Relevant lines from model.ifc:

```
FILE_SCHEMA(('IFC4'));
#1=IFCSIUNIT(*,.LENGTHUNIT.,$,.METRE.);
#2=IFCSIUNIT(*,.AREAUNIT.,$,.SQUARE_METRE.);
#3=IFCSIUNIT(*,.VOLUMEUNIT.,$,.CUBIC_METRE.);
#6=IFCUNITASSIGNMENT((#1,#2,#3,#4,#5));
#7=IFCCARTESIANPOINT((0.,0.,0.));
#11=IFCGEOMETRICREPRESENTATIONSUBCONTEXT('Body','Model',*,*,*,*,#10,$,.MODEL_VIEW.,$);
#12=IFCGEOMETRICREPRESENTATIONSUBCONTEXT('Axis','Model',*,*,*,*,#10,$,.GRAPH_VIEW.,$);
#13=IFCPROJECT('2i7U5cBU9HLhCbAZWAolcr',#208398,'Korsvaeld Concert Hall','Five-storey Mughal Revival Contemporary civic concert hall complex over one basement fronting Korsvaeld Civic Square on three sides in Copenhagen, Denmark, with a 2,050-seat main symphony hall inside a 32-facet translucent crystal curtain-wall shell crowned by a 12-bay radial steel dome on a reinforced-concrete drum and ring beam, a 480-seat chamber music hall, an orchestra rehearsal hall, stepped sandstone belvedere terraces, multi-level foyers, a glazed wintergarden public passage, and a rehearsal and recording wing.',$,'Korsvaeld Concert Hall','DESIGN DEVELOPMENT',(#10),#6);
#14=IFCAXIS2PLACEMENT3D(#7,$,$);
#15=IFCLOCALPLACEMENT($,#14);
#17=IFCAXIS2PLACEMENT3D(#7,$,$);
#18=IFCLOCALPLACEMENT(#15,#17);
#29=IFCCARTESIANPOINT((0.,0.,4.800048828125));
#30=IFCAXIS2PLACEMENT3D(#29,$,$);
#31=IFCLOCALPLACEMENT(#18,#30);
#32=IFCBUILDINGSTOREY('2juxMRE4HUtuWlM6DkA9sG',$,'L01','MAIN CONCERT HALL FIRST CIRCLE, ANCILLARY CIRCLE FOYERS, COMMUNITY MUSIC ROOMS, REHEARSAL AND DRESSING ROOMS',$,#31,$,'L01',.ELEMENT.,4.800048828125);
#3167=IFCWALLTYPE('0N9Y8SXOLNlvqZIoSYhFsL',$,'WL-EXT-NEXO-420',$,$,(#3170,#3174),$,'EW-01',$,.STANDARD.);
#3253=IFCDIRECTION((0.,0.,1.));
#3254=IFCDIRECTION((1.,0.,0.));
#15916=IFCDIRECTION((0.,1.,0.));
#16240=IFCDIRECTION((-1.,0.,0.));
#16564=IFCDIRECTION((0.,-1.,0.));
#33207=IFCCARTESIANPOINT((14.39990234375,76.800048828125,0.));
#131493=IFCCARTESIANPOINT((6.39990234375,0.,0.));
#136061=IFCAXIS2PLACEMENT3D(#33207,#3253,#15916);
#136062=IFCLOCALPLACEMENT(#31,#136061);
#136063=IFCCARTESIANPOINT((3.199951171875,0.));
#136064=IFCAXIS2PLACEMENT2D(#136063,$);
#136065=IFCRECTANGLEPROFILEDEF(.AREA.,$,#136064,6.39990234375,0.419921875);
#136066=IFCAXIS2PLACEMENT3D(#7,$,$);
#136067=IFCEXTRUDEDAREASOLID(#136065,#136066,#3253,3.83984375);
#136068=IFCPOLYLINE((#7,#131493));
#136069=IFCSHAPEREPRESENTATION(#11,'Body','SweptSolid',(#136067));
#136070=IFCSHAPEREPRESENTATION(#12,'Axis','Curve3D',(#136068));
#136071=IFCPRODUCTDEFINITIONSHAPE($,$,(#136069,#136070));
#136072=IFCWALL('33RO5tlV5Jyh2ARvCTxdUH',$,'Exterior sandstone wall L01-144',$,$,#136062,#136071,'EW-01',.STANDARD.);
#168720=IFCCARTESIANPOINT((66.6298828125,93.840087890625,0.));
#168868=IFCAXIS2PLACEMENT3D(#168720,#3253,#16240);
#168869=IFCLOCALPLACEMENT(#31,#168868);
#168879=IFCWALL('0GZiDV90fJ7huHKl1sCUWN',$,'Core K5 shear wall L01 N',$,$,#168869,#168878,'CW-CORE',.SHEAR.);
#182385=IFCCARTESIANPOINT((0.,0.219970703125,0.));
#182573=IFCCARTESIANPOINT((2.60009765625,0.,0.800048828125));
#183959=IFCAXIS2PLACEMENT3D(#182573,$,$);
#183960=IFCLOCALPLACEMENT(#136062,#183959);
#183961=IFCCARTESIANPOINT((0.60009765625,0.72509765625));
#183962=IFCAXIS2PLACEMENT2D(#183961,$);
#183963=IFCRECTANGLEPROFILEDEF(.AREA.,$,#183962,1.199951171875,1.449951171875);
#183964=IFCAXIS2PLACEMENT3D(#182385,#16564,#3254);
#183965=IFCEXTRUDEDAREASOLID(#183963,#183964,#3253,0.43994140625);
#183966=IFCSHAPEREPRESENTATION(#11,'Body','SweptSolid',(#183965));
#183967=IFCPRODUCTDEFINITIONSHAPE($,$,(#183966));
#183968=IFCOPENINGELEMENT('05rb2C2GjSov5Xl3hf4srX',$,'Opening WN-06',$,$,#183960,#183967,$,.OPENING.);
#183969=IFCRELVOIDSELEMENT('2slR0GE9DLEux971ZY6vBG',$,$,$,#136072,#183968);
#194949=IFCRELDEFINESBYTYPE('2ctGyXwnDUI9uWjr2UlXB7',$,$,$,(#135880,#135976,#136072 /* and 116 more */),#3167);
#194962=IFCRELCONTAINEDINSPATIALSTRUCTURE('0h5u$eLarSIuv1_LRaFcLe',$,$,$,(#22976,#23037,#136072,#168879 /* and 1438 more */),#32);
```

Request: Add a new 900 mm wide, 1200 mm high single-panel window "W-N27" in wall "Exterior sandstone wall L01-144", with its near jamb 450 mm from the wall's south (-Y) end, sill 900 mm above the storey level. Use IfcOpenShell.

```python
import numpy as np
import ifcopenshell
import ifcopenshell.api.feature
import ifcopenshell.api.geometry
import ifcopenshell.api.root
import ifcopenshell.api.spatial
import ifcopenshell.geom
import ifcopenshell.util.element
import ifcopenshell.util.placement
import ifcopenshell.util.representation
import ifcopenshell.util.shape
import ifcopenshell.util.unit

model = ifcopenshell.open("model.ifc")
unit_scale = ifcopenshell.util.unit.calculate_unit_scale(model)
settings = ifcopenshell.geom.settings()


def volume(element):
    """Net volume in cubic metres, openings subtracted."""
    shape = ifcopenshell.geom.create_shape(settings, element)
    return ifcopenshell.util.shape.get_volume(shape.geometry)


wall = model.by_guid("33RO5tlV5Jyh2ARvCTxdUH")
storey = ifcopenshell.util.element.get_container(wall, ifc_class="IfcBuildingStorey")
context = ifcopenshell.util.representation.get_context(model, "Model", "Body", "MODEL_VIEW")
before = volume(wall)

width, height, from_end, sill = 0.9, 1.2, 0.45, 0.9  # metres

# The wall runs along its own X axis, and the end named is its -X end.
wall_shape = ifcopenshell.geom.create_shape(settings, wall)
x, y, z = ifcopenshell.util.shape.get_vertices(wall_shape.geometry).T
start = x.min() + from_end
face, thickness = float(y.min()), float(y.max() - y.min())
wall_matrix = ifcopenshell.util.placement.get_local_placement(wall.ObjectPlacement)
level = ifcopenshell.util.placement.get_local_placement(storey.ObjectPlacement)[2, 3]


def in_wall(x, y):
    """Placement at x, y metres in the wall's axes, at sill height."""
    matrix = wall_matrix.copy()
    matrix[:, 3] = wall_matrix @ np.array([x / unit_scale, y / unit_scale, 0.0, 1.0])
    matrix[2, 3] = level + sill / unit_scale
    return matrix


# Opening: a box that overshoots both wall faces by 50 mm.
opening = ifcopenshell.api.root.create_entity(model, ifc_class="IfcOpeningElement", predefined_type="OPENING")
box = ifcopenshell.api.geometry.add_wall_representation(
    model, context=context, length=width, height=height, thickness=thickness + 0.1
)
ifcopenshell.api.geometry.assign_representation(model, product=opening, representation=box)
ifcopenshell.api.geometry.edit_object_placement(model, product=opening, matrix=in_wall(start, face - 0.05), is_si=False)
ifcopenshell.api.feature.add_feature(model, feature=opening, element=wall)

window = ifcopenshell.api.root.create_entity(model, ifc_class="IfcWindow", name="W-N27", predefined_type="WINDOW")
window.OverallWidth, window.OverallHeight = width / unit_scale, height / unit_scale
window.PartitioningType = "SINGLE_PANEL"
body = ifcopenshell.api.geometry.add_window_representation(
    model,
    context=context,
    overall_width=window.OverallWidth,
    overall_height=window.OverallHeight,
    partition_type="SINGLE_PANEL",
)
ifcopenshell.api.geometry.assign_representation(model, product=window, representation=body)
ifcopenshell.api.spatial.assign_container(model, products=[window], relating_structure=storey)
ifcopenshell.api.feature.add_filling(model, opening=opening, element=window)

# Centre the window in the wall's thickness.
ifcopenshell.api.geometry.edit_object_placement(model, product=window, matrix=in_wall(start, face), is_si=False)
window_shape = ifcopenshell.geom.create_shape(settings, window)
depth = ifcopenshell.util.shape.get_vertices(window_shape.geometry)[:, 1]
offset = face + thickness / 2 - (depth.min() + depth.max()) / 2
ifcopenshell.api.geometry.edit_object_placement(model, product=window, matrix=in_wall(start, offset), is_si=False)

after = volume(wall)

print(f"wall volume {before:.3f} -> {after:.3f} m3")

model.write("model_edited.ifc")
```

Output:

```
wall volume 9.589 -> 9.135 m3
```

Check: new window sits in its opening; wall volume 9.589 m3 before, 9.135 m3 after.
